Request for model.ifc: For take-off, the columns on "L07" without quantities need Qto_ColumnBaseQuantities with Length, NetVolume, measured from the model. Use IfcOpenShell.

First a look at what the model holds.

```python
import ifcopenshell
import ifcopenshell.util.element
import ifcopenshell.util.unit

model = ifcopenshell.open("model.ifc")
print(model.schema)
for unit_type in ("LENGTHUNIT", "AREAUNIT", "VOLUMEUNIT"):
    print(unit_type, ifcopenshell.util.unit.calculate_unit_scale(model, unit_type))
storey = next(s for s in model.by_type("IfcBuildingStorey") if s.Name == "L07")
columns = [e for e in ifcopenshell.util.element.get_decomposition(storey) if e.is_a("IfcColumn")]
for e in sorted(columns, key=lambda e: e.id()):
    print(e.id(), e.is_a(), e.Name, list(ifcopenshell.util.element.get_psets(e, qtos_only=True)), sep=" | ")
```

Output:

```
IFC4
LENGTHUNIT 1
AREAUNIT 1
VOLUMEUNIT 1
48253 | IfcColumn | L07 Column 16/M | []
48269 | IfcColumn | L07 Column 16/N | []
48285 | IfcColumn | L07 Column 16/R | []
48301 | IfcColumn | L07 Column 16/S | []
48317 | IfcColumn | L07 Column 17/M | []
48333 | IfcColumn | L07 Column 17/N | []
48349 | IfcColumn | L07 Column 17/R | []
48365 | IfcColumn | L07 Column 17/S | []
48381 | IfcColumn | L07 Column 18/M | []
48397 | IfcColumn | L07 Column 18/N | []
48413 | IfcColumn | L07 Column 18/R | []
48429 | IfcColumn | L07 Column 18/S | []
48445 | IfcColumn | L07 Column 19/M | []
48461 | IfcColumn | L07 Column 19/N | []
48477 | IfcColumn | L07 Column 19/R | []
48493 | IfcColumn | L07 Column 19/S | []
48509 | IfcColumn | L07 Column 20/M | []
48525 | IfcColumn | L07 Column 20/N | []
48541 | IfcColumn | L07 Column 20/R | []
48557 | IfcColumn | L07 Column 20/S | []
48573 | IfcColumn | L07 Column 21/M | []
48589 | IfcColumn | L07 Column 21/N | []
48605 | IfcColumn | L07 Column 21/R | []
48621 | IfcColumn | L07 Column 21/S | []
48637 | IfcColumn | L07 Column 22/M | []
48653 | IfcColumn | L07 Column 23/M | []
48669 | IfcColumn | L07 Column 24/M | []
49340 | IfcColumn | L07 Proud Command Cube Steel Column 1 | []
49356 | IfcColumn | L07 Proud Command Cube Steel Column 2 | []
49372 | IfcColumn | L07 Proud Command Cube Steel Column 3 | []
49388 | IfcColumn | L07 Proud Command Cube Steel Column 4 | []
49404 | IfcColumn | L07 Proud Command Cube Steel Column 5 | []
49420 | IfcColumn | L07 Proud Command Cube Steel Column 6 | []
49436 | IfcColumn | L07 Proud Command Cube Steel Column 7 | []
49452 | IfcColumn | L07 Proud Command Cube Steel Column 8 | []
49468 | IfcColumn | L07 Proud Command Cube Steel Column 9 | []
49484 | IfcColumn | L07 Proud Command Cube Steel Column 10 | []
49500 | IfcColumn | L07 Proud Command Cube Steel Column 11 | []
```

```python
import ifcopenshell
import ifcopenshell.api.pset
import ifcopenshell.geom
import ifcopenshell.util.element
import ifcopenshell.util.shape
import ifcopenshell.util.unit

model = ifcopenshell.open("model.ifc")
unit_scale = ifcopenshell.util.unit.calculate_unit_scale(model)
volume_scale = ifcopenshell.util.unit.calculate_unit_scale(model, "VOLUMEUNIT")
settings = ifcopenshell.geom.settings()

storey = next(s for s in model.by_type("IfcBuildingStorey") if s.Name == "L07")
columns = [e for e in ifcopenshell.util.element.get_decomposition(storey) if e.is_a("IfcColumn")]

for e in sorted(columns, key=lambda e: e.id()):
    if ifcopenshell.util.element.get_psets(e, qtos_only=True, should_inherit=False):
        continue
    # Geometry comes back in metres, in the element's own axes.
    shape = ifcopenshell.geom.create_shape(settings, e)
    values = {
        "Length": ifcopenshell.util.shape.get_z(shape.geometry) / unit_scale,
        "NetVolume": ifcopenshell.util.shape.get_volume(shape.geometry) / volume_scale,
    }
    qto = ifcopenshell.api.pset.add_qto(model, product=e, name="Qto_ColumnBaseQuantities")
    ifcopenshell.api.pset.edit_qto(model, qto=qto, properties=values)
    print(e.id(), {k: round(v, 3) for k, v in values.items()})

model.write("model_edited.ifc")
```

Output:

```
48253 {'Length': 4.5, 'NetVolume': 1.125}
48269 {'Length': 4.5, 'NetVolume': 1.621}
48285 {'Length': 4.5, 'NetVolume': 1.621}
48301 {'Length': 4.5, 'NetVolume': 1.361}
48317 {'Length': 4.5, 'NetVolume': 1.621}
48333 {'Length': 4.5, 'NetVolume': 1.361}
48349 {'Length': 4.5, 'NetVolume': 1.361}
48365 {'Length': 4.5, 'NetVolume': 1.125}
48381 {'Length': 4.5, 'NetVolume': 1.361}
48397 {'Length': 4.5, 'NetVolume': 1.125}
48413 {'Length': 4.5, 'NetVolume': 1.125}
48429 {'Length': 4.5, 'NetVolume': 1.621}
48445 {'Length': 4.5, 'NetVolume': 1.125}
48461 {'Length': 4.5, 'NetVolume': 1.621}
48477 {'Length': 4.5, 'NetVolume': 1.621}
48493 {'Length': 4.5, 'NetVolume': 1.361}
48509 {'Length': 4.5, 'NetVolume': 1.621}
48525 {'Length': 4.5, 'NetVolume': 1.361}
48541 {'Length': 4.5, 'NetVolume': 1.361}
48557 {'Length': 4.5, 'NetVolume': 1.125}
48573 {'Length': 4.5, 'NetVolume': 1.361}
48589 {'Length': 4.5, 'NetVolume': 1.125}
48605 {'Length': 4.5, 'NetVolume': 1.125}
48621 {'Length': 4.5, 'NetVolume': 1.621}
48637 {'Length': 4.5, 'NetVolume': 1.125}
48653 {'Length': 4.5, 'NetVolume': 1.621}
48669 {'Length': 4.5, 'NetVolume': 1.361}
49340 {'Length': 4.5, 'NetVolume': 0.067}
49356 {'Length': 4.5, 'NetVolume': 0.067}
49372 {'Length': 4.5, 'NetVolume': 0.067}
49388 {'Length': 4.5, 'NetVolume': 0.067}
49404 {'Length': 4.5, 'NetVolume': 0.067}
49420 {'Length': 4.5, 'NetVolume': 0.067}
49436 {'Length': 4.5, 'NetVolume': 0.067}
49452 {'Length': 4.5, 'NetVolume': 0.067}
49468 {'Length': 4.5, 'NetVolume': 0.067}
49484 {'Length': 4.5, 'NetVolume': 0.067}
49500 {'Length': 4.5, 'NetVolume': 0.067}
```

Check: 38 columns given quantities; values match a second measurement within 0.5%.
